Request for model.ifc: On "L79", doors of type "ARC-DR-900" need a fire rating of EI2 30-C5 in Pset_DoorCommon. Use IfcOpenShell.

First a look at what the model holds.

```python
import ifcopenshell
import ifcopenshell.util.element

model = ifcopenshell.open("model.ifc")
print(model.schema)
storey = next(s for s in model.by_type("IfcBuildingStorey") if s.Name == "L79")
doors = [e for e in ifcopenshell.util.element.get_decomposition(storey) if e.is_a("IfcDoor")]
seen = {}
for e in doors:
    element_type = ifcopenshell.util.element.get_type(e)
    key = (element_type.Name if element_type != e and element_type else None, ifcopenshell.util.element.get_pset(e, "Pset_DoorCommon", "FireRating"))
    seen[key] = seen.get(key, 0) + 1
for (name, value), count in sorted(seen.items(), key=str):
    print(count, "x", name, "|", value)
```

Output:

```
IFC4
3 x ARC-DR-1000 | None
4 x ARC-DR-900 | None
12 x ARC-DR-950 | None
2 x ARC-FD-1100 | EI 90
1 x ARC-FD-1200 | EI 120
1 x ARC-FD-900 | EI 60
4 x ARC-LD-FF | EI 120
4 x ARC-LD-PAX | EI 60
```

```python
import ifcopenshell
import ifcopenshell.api.pset
import ifcopenshell.util.element

model = ifcopenshell.open("model.ifc")

storey = next(s for s in model.by_type("IfcBuildingStorey") if s.Name == "L79")
doors = [e for e in ifcopenshell.util.element.get_decomposition(storey) if e.is_a("IfcDoor")]

count = 0
for e in doors:
    element_type = ifcopenshell.util.element.get_type(e)
    if element_type in (None, e) or element_type.Name != "ARC-DR-900":
        continue
    found = ifcopenshell.util.element.get_pset(e, "Pset_DoorCommon", should_inherit=False)
    if found:
        pset = model.by_id(found["id"])
        if len(ifcopenshell.util.element.get_elements_by_pset(pset)) > 1:
            pset = ifcopenshell.api.pset.unshare_pset(model, products=[e], pset=pset)[0]
    else:
        pset = ifcopenshell.api.pset.add_pset(model, product=e, name="Pset_DoorCommon")
    ifcopenshell.api.pset.edit_pset(model, pset=pset, properties={"FireRating": "EI2 30-C5"})
    count += 1

print(count, "doors updated")

model.write("model-out.ifc")
```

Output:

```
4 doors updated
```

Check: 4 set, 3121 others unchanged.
